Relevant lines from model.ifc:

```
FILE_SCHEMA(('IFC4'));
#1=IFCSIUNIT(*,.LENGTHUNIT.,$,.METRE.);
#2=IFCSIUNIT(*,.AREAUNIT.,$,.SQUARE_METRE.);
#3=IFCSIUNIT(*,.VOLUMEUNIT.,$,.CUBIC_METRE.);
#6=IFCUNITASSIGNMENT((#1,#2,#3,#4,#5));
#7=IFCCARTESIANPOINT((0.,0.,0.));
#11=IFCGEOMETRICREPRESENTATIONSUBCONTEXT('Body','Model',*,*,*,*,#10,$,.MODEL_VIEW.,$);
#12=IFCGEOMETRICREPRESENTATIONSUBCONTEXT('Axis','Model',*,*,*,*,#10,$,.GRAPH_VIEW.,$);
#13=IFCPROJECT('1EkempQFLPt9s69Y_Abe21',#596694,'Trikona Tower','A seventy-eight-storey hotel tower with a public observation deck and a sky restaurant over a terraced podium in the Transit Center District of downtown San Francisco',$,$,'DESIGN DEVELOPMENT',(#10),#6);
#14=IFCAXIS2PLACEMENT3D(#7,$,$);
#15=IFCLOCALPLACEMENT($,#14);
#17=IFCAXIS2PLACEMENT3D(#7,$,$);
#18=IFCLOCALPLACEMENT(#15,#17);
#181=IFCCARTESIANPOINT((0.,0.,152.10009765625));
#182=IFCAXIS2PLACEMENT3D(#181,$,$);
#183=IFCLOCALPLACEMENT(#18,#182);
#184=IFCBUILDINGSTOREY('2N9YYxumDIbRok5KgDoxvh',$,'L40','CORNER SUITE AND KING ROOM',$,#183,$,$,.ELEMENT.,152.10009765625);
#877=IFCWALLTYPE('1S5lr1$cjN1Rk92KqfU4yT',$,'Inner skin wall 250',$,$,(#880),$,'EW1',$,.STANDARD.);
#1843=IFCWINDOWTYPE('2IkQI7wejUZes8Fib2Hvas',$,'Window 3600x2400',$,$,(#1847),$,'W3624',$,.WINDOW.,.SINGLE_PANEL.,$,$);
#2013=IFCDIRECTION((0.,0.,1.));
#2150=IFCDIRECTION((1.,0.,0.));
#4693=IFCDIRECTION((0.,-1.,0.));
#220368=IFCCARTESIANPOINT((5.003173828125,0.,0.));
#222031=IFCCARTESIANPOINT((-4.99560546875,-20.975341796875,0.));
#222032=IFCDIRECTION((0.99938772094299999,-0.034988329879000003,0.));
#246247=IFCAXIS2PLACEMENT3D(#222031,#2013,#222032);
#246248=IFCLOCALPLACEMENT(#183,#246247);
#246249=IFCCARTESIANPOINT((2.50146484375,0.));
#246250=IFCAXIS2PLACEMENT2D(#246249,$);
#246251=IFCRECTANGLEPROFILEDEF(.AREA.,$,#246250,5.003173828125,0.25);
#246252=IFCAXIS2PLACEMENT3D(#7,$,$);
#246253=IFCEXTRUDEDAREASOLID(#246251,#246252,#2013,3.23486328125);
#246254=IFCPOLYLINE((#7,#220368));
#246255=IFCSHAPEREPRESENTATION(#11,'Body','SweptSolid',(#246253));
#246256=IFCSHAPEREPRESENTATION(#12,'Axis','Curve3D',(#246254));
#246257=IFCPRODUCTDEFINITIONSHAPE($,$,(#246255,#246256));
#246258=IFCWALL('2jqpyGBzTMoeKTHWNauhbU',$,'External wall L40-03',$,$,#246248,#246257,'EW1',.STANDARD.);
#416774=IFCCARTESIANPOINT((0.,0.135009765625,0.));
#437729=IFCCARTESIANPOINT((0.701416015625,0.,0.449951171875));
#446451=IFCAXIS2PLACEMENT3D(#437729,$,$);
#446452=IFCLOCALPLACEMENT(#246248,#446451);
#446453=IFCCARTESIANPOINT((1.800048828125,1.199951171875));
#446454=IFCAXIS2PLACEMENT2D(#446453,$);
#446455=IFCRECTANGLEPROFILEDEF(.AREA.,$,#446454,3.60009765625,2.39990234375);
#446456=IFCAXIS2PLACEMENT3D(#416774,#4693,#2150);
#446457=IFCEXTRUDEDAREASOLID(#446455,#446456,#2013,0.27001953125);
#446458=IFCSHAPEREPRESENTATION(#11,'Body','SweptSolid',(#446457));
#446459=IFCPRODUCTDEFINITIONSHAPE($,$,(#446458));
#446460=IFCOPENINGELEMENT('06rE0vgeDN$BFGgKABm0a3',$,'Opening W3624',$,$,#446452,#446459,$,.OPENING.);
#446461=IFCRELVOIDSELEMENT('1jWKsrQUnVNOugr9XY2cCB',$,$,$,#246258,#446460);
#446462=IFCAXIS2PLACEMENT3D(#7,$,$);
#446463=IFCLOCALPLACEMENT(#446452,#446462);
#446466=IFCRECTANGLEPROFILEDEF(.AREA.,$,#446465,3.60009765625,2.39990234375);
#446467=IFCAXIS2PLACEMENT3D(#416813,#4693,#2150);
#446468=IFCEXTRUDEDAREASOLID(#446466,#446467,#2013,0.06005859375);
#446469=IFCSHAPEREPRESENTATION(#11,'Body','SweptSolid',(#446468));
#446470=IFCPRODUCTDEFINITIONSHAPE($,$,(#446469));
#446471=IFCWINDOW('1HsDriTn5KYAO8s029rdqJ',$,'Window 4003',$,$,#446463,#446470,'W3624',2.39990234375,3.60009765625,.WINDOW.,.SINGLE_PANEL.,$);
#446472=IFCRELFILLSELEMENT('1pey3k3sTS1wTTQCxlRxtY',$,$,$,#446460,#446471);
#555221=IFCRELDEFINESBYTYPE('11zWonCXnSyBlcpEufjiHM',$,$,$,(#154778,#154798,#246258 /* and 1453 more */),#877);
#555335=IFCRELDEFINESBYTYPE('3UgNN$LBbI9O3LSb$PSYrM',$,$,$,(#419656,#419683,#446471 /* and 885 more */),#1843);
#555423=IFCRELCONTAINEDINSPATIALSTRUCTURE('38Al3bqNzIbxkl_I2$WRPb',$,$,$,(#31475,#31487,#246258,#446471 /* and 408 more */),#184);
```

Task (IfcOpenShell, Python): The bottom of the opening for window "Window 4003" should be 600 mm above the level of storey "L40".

```python
import numpy as np
import ifcopenshell
import ifcopenshell.api.geometry
import ifcopenshell.geom
import ifcopenshell.util.element
import ifcopenshell.util.placement
import ifcopenshell.util.shape
import ifcopenshell.util.unit

model = ifcopenshell.open("model.ifc")
unit_scale = ifcopenshell.util.unit.calculate_unit_scale(model)

window = model.by_id(446471)
opening = window.FillsVoids[0].RelatingOpeningElement
storey = ifcopenshell.util.element.get_container(window, ifc_class="IfcBuildingStorey")
level = ifcopenshell.util.placement.get_local_placement(storey.ObjectPlacement)[2, 3]

# The opening's origin need not be at the sill, so measure its lowest point.
shape = ifcopenshell.geom.create_shape(ifcopenshell.geom.settings(), opening)
bottom = ifcopenshell.util.shape.get_shape_bottom_elevation(shape, shape.geometry) / unit_scale
dz = level + 0.6 / unit_scale - bottom

shift = np.array([0.0, 0.0, dz])
# The window is placed relative to its opening, so it follows when the opening moves.
matrix = ifcopenshell.util.placement.get_local_placement(opening.ObjectPlacement)
matrix[:3, 3] += shift
ifcopenshell.api.geometry.edit_object_placement(
    model, product=opening, matrix=matrix, is_si=False, should_transform_children=True
)

print(f"moved by {dz * unit_scale:+.3f} m")

model.write("model_edited.ifc")
```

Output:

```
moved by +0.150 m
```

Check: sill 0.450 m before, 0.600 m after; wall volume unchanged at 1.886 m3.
